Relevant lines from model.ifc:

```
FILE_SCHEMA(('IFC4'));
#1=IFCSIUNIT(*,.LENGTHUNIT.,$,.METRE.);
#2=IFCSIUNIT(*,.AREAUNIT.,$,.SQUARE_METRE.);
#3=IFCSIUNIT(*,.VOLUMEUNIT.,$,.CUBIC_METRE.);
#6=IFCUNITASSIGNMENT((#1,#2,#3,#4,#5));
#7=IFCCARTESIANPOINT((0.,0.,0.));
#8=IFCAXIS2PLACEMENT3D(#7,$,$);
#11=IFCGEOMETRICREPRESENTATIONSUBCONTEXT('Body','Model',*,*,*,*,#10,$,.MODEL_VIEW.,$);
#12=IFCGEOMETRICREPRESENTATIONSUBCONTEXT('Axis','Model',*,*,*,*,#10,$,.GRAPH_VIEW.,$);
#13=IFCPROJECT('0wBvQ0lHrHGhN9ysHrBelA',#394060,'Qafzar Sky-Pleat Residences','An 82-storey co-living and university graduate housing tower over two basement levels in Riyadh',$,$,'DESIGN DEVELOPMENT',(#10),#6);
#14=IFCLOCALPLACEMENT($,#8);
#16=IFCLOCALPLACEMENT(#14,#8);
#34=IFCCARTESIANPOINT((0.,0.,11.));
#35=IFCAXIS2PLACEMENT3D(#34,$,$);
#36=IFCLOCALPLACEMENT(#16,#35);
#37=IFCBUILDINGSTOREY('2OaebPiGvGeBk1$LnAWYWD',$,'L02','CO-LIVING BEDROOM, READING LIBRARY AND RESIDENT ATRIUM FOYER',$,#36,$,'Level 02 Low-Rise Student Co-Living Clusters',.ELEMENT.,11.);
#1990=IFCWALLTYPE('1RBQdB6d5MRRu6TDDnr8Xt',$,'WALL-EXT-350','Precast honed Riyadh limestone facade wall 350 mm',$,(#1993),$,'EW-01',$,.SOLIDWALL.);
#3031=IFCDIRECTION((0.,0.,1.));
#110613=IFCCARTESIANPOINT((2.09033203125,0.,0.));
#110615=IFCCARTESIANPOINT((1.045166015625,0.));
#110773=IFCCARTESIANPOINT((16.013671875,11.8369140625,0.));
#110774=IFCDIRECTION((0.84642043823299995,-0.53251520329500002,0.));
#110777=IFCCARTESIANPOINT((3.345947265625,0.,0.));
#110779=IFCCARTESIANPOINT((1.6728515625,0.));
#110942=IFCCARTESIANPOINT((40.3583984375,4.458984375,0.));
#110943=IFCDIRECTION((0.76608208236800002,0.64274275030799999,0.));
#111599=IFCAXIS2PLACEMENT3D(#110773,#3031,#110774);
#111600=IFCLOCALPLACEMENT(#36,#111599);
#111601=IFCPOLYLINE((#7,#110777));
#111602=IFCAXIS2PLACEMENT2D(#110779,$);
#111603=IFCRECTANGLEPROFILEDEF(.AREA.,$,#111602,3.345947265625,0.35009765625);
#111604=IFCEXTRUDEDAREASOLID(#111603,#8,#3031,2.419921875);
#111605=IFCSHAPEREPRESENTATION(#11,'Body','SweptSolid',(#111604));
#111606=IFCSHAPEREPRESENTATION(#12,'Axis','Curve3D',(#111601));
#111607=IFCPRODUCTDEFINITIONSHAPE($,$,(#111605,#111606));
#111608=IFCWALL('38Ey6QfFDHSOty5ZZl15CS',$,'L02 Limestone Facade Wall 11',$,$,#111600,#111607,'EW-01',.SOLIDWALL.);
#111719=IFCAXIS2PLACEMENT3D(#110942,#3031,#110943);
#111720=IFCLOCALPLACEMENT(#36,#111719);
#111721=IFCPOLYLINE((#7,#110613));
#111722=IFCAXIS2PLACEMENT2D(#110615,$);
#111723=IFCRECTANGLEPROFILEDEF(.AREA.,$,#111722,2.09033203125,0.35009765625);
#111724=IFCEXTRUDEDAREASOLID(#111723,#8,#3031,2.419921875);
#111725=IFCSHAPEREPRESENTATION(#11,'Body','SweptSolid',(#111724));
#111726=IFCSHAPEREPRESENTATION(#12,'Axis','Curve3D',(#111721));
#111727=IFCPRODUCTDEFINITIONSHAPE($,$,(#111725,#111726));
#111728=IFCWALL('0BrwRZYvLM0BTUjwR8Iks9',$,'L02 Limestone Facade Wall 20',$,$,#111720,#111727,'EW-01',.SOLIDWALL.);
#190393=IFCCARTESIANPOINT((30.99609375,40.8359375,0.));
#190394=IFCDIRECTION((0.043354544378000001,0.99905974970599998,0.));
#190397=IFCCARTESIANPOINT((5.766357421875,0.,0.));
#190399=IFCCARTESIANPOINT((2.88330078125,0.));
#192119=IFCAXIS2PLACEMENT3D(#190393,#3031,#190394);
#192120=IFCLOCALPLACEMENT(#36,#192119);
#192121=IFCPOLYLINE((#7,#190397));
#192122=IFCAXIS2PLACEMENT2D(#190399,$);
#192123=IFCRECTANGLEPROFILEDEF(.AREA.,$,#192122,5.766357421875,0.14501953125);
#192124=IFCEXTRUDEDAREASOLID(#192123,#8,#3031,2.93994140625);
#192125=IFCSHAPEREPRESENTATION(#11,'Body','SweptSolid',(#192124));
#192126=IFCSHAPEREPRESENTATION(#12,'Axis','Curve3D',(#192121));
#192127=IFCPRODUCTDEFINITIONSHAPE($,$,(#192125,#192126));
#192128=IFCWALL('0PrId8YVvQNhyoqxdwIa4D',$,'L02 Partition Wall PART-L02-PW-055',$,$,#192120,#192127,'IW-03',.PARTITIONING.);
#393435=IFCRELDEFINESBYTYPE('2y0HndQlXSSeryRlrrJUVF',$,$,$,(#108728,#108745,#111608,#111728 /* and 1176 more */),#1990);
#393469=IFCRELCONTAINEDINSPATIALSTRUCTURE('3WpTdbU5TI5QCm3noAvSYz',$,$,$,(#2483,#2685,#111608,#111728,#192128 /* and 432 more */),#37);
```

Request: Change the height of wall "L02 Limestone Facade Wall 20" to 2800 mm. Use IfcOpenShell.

```python
import ifcopenshell
import ifcopenshell.geom
import ifcopenshell.util.representation
import ifcopenshell.util.shape

model = ifcopenshell.open("model.ifc")
settings = ifcopenshell.geom.settings()


def volume(element):
    """Net volume in cubic metres, openings subtracted."""
    shape = ifcopenshell.geom.create_shape(settings, element)
    return ifcopenshell.util.shape.get_volume(shape.geometry)


wall = model.by_guid("0BrwRZYvLM0BTUjwR8Iks9")
before = volume(wall)

body = ifcopenshell.util.representation.get_representation(wall, "Model", "Body")
solid = body.Items[0]
old_height = solid.Depth
solid.Depth = 2.8
after = volume(wall)

print(f"height {old_height:g} -> {solid.Depth:g}, volume {before:.3f} -> {after:.3f} m3")

model.write("model_updated.ifc")
```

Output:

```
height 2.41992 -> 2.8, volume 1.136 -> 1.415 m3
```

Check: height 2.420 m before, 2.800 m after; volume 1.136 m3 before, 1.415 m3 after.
